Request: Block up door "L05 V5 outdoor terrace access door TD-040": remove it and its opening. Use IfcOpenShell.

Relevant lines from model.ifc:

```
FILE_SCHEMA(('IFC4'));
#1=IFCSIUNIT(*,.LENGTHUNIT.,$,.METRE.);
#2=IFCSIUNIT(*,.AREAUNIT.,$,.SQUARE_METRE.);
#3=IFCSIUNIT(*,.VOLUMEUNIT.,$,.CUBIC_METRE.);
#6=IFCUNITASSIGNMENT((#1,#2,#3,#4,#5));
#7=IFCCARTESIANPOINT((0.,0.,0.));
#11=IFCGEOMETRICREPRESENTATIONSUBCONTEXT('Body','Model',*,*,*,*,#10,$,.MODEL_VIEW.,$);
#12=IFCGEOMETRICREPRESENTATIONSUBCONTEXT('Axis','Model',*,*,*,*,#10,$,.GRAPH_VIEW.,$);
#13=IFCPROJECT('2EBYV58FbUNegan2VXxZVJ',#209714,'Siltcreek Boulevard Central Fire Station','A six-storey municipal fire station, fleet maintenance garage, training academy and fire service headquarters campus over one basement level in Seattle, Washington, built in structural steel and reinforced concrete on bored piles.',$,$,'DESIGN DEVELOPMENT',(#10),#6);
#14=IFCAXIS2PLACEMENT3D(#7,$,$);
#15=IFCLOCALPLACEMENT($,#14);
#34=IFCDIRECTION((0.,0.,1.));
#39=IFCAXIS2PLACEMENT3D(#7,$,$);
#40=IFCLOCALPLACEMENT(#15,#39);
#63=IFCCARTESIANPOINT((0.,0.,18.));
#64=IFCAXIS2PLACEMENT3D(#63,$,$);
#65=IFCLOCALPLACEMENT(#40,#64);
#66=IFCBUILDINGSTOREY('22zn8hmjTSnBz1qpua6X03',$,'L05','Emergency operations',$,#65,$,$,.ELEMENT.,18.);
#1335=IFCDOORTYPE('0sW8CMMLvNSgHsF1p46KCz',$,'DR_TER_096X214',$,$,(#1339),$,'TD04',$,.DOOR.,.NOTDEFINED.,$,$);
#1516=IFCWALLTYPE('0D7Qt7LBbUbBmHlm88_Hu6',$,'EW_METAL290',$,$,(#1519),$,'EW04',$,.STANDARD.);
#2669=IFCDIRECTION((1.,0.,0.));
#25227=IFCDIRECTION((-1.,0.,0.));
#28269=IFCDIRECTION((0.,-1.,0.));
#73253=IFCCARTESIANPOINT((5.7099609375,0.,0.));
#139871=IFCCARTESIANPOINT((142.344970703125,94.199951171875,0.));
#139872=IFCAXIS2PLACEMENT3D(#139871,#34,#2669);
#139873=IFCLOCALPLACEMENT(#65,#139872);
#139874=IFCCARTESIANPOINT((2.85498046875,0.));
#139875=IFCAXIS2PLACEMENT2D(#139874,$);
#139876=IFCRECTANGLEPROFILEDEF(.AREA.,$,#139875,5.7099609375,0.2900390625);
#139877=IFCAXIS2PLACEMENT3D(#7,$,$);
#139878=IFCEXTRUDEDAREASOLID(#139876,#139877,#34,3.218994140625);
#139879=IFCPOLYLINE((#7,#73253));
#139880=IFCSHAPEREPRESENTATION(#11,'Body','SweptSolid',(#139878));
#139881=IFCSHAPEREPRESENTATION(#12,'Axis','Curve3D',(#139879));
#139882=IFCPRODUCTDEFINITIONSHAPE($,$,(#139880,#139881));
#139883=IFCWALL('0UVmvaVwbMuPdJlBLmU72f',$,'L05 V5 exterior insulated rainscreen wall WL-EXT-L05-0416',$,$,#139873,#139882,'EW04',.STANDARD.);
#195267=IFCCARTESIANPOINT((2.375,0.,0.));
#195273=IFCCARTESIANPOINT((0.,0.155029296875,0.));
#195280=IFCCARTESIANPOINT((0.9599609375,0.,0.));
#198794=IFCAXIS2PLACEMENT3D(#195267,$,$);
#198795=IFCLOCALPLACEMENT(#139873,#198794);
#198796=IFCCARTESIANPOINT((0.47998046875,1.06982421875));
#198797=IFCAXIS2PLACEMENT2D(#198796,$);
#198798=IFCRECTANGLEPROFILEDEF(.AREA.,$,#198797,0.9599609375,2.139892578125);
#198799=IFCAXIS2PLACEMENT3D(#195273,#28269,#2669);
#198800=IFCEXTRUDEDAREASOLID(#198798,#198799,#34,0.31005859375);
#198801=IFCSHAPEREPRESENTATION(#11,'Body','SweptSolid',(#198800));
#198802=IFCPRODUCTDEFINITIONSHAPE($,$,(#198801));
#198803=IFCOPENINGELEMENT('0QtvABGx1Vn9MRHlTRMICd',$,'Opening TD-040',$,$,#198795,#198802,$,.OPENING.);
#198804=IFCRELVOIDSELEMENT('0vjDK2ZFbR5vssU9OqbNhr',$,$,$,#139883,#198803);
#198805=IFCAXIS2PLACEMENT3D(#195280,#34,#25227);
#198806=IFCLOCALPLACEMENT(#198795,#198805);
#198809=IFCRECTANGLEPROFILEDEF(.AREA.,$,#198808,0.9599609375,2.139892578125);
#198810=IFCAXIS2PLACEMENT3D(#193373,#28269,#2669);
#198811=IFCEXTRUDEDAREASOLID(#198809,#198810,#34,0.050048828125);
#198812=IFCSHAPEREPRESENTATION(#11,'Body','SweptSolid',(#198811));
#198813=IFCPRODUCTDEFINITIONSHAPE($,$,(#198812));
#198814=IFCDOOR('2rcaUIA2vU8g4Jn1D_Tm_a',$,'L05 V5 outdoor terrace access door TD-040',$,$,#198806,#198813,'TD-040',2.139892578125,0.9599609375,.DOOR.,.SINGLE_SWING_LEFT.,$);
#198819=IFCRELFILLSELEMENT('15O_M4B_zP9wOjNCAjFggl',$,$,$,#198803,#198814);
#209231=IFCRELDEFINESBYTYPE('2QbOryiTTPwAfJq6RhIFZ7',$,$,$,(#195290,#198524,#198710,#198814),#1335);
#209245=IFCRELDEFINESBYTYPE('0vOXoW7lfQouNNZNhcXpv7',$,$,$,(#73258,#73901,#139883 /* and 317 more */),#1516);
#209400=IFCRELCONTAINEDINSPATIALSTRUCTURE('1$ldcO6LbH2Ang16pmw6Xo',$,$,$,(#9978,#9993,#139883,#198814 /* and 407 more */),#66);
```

```python
import ifcopenshell
import ifcopenshell.api.feature
import ifcopenshell.api.root
import ifcopenshell.geom
import ifcopenshell.util.shape

model = ifcopenshell.open("model.ifc")
settings = ifcopenshell.geom.settings()


def volume(element):
    """Net volume in cubic metres, openings subtracted."""
    shape = ifcopenshell.geom.create_shape(settings, element)
    return ifcopenshell.util.shape.get_volume(shape.geometry)


door = model.by_guid("2rcaUIA2vU8g4Jn1D_Tm_a")
opening = door.FillsVoids[0].RelatingOpeningElement
wall = opening.VoidsElements[0].RelatingBuildingElement
before = volume(wall)

ifcopenshell.api.root.remove_product(model, product=door)
ifcopenshell.api.feature.remove_feature(model, feature=opening)

after = volume(wall)

print(f"wall volume {before:.3f} -> {after:.3f} m3")

model.write("model_updated.ifc")
```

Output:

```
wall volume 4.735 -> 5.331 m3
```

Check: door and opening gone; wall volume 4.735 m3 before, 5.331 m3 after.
